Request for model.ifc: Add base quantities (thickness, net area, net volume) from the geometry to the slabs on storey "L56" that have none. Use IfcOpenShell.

First a look at what the model holds.

```python
import ifcopenshell
import ifcopenshell.util.element
import ifcopenshell.util.unit

model = ifcopenshell.open("model.ifc")
print(model.schema)
for unit_type in ("LENGTHUNIT", "AREAUNIT", "VOLUMEUNIT"):
    print(unit_type, ifcopenshell.util.unit.calculate_unit_scale(model, unit_type))
storey = next(s for s in model.by_type("IfcBuildingStorey") if s.Name == "L56")
slabs = [e for e in ifcopenshell.util.element.get_decomposition(storey) if e.is_a("IfcSlab")]
for e in sorted(slabs, key=lambda e: e.id()):
    print(e.id(), e.is_a(), e.Name, list(ifcopenshell.util.element.get_psets(e, qtos_only=True)), sep=" | ")
```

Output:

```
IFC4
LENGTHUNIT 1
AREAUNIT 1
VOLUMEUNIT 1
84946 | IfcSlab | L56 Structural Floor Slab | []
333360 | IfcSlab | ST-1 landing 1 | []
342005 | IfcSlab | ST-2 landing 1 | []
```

```python
import ifcopenshell
import ifcopenshell.api.pset
import ifcopenshell.geom
import ifcopenshell.util.element
import ifcopenshell.util.shape
import ifcopenshell.util.unit

model = ifcopenshell.open("model.ifc")
unit_scale = ifcopenshell.util.unit.calculate_unit_scale(model)
area_scale = ifcopenshell.util.unit.calculate_unit_scale(model, "AREAUNIT")
volume_scale = ifcopenshell.util.unit.calculate_unit_scale(model, "VOLUMEUNIT")
settings = ifcopenshell.geom.settings()

storey = next(s for s in model.by_type("IfcBuildingStorey") if s.Name == "L56")
slabs = [e for e in ifcopenshell.util.element.get_decomposition(storey) if e.is_a("IfcSlab")]

for e in sorted(slabs, key=lambda e: e.id()):
    if ifcopenshell.util.element.get_psets(e, qtos_only=True, should_inherit=False):
        continue
    # Geometry comes back in metres, in the element's own axes.
    shape = ifcopenshell.geom.create_shape(settings, e)
    values = {
        "Width": ifcopenshell.util.shape.get_z(shape.geometry) / unit_scale,
        "NetArea": ifcopenshell.util.shape.get_footprint_area(shape.geometry) / area_scale,
        "NetVolume": ifcopenshell.util.shape.get_volume(shape.geometry) / volume_scale,
    }
    qto = ifcopenshell.api.pset.add_qto(model, product=e, name="Qto_SlabBaseQuantities")
    ifcopenshell.api.pset.edit_qto(model, qto=qto, properties=values)
    print(e.id(), {k: round(v, 3) for k, v in values.items()})

model.write("model_updated.ifc")
```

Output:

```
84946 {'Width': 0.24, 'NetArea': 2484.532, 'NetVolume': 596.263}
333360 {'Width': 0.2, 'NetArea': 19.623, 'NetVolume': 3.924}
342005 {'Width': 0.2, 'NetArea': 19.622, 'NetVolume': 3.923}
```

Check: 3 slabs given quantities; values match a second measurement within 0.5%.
